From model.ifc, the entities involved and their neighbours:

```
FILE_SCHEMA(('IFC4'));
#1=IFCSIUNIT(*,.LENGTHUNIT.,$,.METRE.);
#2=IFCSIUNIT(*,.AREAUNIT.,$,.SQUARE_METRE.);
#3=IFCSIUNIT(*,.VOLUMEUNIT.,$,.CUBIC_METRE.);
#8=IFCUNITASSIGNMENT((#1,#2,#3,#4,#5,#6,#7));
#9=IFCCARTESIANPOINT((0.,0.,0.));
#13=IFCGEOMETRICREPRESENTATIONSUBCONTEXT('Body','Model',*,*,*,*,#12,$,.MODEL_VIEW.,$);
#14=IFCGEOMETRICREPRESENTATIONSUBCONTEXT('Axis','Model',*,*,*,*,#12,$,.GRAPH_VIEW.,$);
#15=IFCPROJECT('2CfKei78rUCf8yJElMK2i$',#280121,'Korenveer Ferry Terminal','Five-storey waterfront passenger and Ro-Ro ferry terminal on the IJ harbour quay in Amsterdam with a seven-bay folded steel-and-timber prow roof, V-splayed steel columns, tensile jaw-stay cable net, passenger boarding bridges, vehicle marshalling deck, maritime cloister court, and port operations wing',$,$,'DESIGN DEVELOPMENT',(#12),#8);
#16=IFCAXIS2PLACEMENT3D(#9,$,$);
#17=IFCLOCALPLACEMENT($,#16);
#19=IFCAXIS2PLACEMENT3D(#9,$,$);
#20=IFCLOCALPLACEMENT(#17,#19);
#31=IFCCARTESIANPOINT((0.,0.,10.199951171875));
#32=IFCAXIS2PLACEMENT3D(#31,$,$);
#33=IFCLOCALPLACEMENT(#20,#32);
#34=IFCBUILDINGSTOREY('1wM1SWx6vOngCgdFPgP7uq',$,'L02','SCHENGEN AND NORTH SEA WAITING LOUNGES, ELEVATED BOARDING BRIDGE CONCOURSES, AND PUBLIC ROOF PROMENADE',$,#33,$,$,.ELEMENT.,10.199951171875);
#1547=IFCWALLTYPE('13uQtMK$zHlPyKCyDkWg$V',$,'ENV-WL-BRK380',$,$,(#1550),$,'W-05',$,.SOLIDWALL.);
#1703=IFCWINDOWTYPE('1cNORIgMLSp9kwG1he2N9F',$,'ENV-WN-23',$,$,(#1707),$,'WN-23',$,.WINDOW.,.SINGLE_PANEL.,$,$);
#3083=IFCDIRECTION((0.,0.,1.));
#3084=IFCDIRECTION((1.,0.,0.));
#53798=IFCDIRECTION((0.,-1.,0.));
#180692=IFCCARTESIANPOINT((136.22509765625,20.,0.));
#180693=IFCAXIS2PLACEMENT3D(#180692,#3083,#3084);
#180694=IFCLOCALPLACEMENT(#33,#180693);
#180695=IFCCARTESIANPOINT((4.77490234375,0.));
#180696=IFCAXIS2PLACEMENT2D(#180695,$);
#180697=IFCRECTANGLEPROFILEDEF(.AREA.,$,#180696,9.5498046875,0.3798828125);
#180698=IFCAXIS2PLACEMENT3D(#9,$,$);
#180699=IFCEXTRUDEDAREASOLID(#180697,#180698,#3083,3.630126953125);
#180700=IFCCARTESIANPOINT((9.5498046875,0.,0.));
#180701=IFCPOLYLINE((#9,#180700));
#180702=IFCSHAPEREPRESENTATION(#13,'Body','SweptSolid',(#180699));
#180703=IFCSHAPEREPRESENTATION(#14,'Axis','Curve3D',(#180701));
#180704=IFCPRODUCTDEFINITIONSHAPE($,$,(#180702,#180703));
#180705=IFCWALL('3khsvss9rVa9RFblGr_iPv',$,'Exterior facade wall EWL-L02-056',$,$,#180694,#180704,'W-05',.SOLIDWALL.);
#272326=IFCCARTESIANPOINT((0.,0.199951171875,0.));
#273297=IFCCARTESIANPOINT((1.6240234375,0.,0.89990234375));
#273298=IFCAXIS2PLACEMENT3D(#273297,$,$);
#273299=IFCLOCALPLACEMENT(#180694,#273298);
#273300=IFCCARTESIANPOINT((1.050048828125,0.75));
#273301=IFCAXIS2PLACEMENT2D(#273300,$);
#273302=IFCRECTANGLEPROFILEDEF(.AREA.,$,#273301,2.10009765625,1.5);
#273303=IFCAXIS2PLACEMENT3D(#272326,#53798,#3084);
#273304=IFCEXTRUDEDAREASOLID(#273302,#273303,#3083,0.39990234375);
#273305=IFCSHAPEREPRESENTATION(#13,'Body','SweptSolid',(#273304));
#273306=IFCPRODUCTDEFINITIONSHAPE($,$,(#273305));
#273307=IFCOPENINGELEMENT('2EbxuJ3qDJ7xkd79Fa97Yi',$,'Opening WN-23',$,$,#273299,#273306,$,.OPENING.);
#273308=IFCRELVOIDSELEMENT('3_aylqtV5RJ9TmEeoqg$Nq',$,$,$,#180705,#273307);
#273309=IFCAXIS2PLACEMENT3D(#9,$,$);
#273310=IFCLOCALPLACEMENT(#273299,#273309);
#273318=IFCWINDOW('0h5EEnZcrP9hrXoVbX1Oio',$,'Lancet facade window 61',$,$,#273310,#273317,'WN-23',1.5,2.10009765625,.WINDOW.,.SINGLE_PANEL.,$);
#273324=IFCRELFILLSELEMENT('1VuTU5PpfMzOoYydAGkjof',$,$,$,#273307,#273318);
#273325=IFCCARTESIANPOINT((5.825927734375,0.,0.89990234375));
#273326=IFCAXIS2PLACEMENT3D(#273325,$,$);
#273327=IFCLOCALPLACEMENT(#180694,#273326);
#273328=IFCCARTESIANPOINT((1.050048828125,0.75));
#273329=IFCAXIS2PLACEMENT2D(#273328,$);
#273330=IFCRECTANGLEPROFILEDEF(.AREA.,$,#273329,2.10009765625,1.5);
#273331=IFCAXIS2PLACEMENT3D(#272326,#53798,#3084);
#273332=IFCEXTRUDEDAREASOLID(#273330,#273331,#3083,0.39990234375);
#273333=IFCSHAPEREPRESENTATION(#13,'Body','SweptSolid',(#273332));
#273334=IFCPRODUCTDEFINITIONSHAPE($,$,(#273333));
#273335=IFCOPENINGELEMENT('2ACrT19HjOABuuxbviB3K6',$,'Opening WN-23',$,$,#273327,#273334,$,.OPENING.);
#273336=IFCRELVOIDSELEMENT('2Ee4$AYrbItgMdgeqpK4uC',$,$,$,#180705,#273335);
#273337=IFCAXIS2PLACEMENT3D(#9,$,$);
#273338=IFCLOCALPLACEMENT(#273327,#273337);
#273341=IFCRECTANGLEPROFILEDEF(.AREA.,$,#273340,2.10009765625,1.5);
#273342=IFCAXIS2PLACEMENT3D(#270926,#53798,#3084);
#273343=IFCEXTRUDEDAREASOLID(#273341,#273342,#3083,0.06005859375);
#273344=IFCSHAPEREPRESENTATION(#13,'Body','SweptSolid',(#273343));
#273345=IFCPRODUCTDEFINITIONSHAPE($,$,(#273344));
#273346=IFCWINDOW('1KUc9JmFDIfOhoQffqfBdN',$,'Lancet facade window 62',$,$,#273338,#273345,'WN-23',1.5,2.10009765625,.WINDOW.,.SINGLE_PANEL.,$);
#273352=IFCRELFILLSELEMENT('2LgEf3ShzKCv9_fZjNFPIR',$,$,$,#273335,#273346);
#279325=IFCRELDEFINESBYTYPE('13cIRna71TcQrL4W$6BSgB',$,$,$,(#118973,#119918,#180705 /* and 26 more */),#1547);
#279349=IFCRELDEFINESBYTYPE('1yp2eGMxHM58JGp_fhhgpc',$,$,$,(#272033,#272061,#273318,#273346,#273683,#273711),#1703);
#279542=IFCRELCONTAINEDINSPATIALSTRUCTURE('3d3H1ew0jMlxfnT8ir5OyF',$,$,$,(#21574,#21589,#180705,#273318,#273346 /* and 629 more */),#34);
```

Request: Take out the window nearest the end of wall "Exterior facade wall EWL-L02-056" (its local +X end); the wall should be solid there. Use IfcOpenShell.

```python
import ifcopenshell
import ifcopenshell.api.feature
import ifcopenshell.api.root
import ifcopenshell.geom
import ifcopenshell.util.shape

model = ifcopenshell.open("model.ifc")
settings = ifcopenshell.geom.settings()


def volume(element):
    """Net volume in cubic metres, openings subtracted."""
    shape = ifcopenshell.geom.create_shape(settings, element)
    return ifcopenshell.util.shape.get_volume(shape.geometry)


window = model.by_guid("1KUc9JmFDIfOhoQffqfBdN")
opening = window.FillsVoids[0].RelatingOpeningElement
wall = opening.VoidsElements[0].RelatingBuildingElement
before = volume(wall)

ifcopenshell.api.root.remove_product(model, product=window)
ifcopenshell.api.feature.remove_feature(model, feature=opening)

after = volume(wall)

print(f"wall volume {before:.3f} -> {after:.3f} m3")

model.write("model_edited.ifc")
```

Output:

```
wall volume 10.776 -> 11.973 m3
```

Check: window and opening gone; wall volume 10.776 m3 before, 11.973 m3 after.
